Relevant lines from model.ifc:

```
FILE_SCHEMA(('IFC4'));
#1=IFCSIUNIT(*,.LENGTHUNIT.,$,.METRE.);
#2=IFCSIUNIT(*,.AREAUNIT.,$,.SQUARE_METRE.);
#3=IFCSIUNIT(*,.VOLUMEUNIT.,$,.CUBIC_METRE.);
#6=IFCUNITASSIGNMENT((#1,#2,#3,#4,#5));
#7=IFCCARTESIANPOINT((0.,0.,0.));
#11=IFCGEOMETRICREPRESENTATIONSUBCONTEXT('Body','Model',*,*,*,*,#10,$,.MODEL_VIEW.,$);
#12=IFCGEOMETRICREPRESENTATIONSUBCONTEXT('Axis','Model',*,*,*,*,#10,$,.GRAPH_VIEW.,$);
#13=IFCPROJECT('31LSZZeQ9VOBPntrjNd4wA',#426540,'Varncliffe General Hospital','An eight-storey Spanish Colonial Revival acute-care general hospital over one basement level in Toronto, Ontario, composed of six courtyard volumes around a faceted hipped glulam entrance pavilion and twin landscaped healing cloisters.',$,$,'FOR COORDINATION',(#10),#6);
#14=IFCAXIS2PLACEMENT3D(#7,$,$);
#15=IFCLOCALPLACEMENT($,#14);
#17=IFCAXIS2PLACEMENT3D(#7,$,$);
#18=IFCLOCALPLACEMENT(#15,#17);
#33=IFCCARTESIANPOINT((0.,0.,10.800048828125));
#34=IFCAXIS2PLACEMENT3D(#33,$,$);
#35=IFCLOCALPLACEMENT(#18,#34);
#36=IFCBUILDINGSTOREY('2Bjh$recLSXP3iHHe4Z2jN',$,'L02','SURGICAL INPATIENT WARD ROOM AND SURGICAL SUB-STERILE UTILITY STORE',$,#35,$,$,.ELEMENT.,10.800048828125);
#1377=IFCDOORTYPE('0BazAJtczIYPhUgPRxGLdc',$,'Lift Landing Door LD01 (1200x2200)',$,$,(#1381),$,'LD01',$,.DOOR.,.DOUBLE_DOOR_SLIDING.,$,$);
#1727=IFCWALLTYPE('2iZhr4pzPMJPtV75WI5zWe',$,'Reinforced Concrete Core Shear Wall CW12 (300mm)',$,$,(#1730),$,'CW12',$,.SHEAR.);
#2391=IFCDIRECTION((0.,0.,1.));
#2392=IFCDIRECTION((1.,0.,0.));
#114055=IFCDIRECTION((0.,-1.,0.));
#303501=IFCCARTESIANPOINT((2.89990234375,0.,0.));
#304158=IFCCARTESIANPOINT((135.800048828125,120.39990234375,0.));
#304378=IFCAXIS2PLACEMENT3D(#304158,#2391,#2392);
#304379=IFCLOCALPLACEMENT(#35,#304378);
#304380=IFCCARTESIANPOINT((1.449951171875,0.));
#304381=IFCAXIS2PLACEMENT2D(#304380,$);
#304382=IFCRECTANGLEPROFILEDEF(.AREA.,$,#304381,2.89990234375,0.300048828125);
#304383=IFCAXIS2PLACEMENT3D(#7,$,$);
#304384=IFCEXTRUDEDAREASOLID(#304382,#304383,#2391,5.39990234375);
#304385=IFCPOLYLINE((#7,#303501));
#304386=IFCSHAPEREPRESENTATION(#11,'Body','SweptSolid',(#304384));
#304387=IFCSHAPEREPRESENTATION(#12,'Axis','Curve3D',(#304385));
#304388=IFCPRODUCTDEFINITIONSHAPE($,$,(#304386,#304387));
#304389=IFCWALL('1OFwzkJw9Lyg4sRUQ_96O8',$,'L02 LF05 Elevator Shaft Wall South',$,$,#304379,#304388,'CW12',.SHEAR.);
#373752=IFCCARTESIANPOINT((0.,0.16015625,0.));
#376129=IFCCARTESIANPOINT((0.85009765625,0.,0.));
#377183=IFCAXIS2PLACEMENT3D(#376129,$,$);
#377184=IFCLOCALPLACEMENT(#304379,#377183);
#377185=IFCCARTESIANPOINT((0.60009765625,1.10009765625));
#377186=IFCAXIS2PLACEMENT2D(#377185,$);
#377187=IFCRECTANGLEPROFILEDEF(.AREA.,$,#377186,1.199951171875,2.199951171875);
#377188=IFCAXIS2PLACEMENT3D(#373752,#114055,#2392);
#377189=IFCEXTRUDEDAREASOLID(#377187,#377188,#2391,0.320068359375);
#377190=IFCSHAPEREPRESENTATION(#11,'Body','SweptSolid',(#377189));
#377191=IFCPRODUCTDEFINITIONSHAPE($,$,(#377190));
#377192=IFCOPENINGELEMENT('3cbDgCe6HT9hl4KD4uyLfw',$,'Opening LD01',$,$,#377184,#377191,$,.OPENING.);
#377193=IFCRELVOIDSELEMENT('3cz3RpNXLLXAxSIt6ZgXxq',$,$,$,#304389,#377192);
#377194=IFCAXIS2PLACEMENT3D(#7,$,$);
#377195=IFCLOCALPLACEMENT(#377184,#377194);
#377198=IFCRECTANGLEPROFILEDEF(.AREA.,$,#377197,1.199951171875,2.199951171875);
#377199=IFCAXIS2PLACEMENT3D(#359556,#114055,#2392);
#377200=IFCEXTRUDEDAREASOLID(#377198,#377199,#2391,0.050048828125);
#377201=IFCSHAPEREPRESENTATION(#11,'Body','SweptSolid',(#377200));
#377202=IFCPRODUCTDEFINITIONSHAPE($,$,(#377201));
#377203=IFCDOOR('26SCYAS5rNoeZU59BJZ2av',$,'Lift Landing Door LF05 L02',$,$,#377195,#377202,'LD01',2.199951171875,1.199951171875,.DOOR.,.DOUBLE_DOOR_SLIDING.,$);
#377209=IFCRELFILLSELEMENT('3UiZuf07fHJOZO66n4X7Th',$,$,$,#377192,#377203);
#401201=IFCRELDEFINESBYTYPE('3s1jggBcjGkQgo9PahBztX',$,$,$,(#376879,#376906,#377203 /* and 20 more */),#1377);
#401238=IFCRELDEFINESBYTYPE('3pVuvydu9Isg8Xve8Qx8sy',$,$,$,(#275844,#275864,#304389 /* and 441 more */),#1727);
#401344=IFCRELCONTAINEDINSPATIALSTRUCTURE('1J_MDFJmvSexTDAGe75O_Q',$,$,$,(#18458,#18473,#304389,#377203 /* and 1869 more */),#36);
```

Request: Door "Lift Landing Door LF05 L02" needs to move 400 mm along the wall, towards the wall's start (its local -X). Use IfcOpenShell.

```python
import ifcopenshell
import ifcopenshell.api.geometry
import ifcopenshell.util.placement
import ifcopenshell.util.unit

model = ifcopenshell.open("model.ifc")
unit_scale = ifcopenshell.util.unit.calculate_unit_scale(model)

door = model.by_guid("26SCYAS5rNoeZU59BJZ2av")
opening = door.FillsVoids[0].RelatingOpeningElement
wall = opening.VoidsElements[0].RelatingBuildingElement

wall_matrix = ifcopenshell.util.placement.get_local_placement(wall.ObjectPlacement)
shift = wall_matrix[:3, 0] * -0.4 / unit_scale
before = ifcopenshell.util.placement.get_local_placement(door.ObjectPlacement)[:3, 3].copy()

# The door is placed relative to its opening, so it follows when the opening moves.
matrix = ifcopenshell.util.placement.get_local_placement(opening.ObjectPlacement)
matrix[:3, 3] += shift
ifcopenshell.api.geometry.edit_object_placement(
    model, product=opening, matrix=matrix, is_si=False, should_transform_children=True
)

after = ifcopenshell.util.placement.get_local_placement(door.ObjectPlacement)[:3, 3]
print("door moved by", (after - before).round(3) + 0.0)

model.write("model-out.ifc")
```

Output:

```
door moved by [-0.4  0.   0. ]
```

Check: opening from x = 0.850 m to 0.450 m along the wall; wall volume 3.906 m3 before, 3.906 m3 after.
